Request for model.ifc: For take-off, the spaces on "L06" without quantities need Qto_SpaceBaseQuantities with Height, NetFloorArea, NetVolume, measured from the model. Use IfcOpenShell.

First a look at what the model holds.

```python
import ifcopenshell
import ifcopenshell.util.element
import ifcopenshell.util.unit

model = ifcopenshell.open("model.ifc")
print(model.schema)
for unit_type in ("LENGTHUNIT", "AREAUNIT", "VOLUMEUNIT"):
    print(unit_type, ifcopenshell.util.unit.calculate_unit_scale(model, unit_type))
storey = next(s for s in model.by_type("IfcBuildingStorey") if s.Name == "L06")
spaces = [e for e in ifcopenshell.util.element.get_decomposition(storey) if e.is_a("IfcSpace")]
for e in sorted(spaces, key=lambda e: e.id()):
    print(e.id(), e.is_a(), e.Name, list(ifcopenshell.util.element.get_psets(e, qtos_only=True)), sep=" | ")
```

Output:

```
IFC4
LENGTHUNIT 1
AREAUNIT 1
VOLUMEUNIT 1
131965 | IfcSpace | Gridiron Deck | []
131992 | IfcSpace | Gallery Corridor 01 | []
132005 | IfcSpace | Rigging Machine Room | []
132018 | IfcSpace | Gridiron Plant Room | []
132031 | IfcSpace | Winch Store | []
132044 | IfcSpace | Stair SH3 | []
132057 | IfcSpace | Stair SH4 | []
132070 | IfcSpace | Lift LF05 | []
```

```python
import ifcopenshell
import ifcopenshell.api.pset
import ifcopenshell.geom
import ifcopenshell.util.element
import ifcopenshell.util.shape
import ifcopenshell.util.unit

model = ifcopenshell.open("model.ifc")
unit_scale = ifcopenshell.util.unit.calculate_unit_scale(model)
area_scale = ifcopenshell.util.unit.calculate_unit_scale(model, "AREAUNIT")
volume_scale = ifcopenshell.util.unit.calculate_unit_scale(model, "VOLUMEUNIT")
settings = ifcopenshell.geom.settings()

storey = next(s for s in model.by_type("IfcBuildingStorey") if s.Name == "L06")
spaces = [e for e in ifcopenshell.util.element.get_decomposition(storey) if e.is_a("IfcSpace")]

for e in sorted(spaces, key=lambda e: e.id()):
    if ifcopenshell.util.element.get_psets(e, qtos_only=True, should_inherit=False):
        continue
    # Geometry comes back in metres, in the element's own axes.
    shape = ifcopenshell.geom.create_shape(settings, e)
    values = {
        "Height": ifcopenshell.util.shape.get_z(shape.geometry) / unit_scale,
        "NetFloorArea": ifcopenshell.util.shape.get_footprint_area(shape.geometry) / area_scale,
        "NetVolume": ifcopenshell.util.shape.get_volume(shape.geometry) / volume_scale,
    }
    qto = ifcopenshell.api.pset.add_qto(model, product=e, name="Qto_SpaceBaseQuantities")
    ifcopenshell.api.pset.edit_qto(model, qto=qto, properties=values)
    print(e.id(), {k: round(v, 3) for k, v in values.items()})

model.write("model_updated.ifc")
```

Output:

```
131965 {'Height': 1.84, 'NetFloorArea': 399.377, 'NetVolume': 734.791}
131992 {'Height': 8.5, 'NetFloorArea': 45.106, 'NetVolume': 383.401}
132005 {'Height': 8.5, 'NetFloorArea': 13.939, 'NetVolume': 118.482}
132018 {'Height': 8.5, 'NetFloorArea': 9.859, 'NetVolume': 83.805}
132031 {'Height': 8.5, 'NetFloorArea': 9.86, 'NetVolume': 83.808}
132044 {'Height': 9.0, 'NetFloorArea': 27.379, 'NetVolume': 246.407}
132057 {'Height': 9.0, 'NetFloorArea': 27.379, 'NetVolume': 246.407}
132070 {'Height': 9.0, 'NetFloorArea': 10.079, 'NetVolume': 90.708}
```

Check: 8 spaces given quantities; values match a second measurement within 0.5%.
